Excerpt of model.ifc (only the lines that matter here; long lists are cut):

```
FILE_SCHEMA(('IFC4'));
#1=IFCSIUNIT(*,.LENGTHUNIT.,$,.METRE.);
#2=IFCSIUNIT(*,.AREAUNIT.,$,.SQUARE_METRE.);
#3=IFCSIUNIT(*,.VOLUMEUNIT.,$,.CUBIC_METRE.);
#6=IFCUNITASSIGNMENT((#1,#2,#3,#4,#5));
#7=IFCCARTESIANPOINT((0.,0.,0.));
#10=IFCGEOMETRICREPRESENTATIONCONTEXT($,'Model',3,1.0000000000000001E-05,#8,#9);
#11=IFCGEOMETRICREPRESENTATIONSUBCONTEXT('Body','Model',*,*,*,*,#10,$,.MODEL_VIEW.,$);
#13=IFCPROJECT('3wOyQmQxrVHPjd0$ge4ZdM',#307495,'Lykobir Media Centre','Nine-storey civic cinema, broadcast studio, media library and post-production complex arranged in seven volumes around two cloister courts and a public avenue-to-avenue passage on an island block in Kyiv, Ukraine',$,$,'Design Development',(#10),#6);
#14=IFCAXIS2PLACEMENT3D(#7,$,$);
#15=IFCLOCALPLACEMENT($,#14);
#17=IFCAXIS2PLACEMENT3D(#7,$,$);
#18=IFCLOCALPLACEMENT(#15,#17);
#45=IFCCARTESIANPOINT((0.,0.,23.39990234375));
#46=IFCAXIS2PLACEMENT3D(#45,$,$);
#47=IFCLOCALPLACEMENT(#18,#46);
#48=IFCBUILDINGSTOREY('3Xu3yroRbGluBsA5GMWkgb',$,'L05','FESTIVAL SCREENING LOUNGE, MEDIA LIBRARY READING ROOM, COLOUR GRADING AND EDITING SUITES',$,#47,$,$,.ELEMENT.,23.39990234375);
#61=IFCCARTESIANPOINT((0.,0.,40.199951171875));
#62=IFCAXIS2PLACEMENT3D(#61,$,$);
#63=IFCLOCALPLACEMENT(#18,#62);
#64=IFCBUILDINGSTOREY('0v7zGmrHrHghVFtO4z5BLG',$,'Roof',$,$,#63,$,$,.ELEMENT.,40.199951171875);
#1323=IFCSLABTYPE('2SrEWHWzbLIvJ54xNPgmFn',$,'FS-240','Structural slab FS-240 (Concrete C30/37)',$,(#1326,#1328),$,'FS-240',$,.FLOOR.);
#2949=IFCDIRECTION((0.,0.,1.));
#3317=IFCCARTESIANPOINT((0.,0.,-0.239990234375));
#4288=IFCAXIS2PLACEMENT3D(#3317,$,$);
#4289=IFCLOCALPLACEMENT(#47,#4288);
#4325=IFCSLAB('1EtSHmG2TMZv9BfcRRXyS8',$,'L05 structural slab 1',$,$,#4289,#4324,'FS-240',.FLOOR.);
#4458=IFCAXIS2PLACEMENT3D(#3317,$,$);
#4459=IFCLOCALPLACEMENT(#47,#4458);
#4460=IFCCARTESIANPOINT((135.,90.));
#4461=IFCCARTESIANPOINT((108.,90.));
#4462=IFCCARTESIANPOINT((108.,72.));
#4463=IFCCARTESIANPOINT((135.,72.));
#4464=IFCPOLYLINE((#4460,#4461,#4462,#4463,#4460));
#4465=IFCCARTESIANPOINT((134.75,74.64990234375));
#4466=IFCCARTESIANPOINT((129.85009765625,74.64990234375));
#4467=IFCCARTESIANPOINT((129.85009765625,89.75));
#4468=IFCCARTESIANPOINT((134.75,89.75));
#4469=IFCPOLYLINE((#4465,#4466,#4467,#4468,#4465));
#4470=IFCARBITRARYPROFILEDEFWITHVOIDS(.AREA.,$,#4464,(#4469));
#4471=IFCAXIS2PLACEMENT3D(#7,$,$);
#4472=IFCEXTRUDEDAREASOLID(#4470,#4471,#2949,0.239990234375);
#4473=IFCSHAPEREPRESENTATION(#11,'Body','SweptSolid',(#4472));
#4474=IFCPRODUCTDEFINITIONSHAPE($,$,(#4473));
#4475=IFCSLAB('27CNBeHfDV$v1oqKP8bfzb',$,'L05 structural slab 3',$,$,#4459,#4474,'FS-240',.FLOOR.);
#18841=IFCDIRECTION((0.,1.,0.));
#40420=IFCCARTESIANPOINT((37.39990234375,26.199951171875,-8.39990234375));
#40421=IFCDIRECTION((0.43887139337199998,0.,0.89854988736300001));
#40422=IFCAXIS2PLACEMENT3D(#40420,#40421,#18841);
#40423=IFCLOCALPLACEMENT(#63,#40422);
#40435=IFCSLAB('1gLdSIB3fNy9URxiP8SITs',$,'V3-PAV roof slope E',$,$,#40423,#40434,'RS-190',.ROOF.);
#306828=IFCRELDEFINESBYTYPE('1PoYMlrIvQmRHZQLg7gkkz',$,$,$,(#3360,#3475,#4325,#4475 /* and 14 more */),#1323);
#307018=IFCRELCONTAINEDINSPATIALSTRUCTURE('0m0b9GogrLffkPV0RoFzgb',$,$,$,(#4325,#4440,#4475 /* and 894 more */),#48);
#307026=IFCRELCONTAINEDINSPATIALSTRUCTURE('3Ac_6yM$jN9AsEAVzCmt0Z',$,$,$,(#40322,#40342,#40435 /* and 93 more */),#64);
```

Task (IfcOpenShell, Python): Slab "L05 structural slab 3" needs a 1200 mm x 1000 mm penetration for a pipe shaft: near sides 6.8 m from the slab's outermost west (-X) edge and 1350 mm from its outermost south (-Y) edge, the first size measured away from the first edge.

```python
import numpy as np
import ifcopenshell
import ifcopenshell.api.feature
import ifcopenshell.api.geometry
import ifcopenshell.api.root
import ifcopenshell.geom
import ifcopenshell.util.placement
import ifcopenshell.util.representation
import ifcopenshell.util.shape
import ifcopenshell.util.unit

model = ifcopenshell.open("model.ifc")
unit_scale = ifcopenshell.util.unit.calculate_unit_scale(model)
settings = ifcopenshell.geom.settings()


def volume(element):
    """Net volume in cubic metres, openings subtracted."""
    shape = ifcopenshell.geom.create_shape(settings, element)
    return ifcopenshell.util.shape.get_volume(shape.geometry)


slab = model.by_guid("27CNBeHfDV$v1oqKP8bfzb")
before = volume(slab)

# Extent in the slab's own axes, in metres. The edges named are its -X and -Y sides.
slab_shape = ifcopenshell.geom.create_shape(settings, slab)
vertices = ifcopenshell.util.shape.get_vertices(slab_shape.geometry)
x_min, y_min, bottom = vertices.min(axis=0)
top = vertices[:, 2].max()

opening = ifcopenshell.api.root.create_entity(model, ifc_class="IfcOpeningElement", name="Pipe shaft opening", predefined_type="OPENING")
context = ifcopenshell.util.representation.get_context(model, "Model", "Body", "MODEL_VIEW")
width, depth = 1.2, 1
outline = [(0.0, 0.0), (width, 0.0), (width, depth), (0.0, depth), (0.0, 0.0)]
# Overshoot both faces by 50 mm so the cut is clean.
shape = ifcopenshell.api.geometry.add_slab_representation(
    model, context=context, depth=top - bottom + 0.1, polyline=outline
)
ifcopenshell.api.geometry.assign_representation(model, product=opening, representation=shape)

matrix = ifcopenshell.util.placement.get_local_placement(slab.ObjectPlacement)
matrix[:, 3] = matrix @ np.append(np.array([x_min + 6.8, y_min + 1.35, bottom - 0.05]) / unit_scale, 1.0)
ifcopenshell.api.geometry.edit_object_placement(model, product=opening, matrix=matrix, is_si=False)
ifcopenshell.api.feature.add_feature(model, feature=opening, element=slab)

after = volume(slab)

print(f"slab volume {before:.3f} -> {after:.3f} m3")

model.write("model_updated.ifc")
```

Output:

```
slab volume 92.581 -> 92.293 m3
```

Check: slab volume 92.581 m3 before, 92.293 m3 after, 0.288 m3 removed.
